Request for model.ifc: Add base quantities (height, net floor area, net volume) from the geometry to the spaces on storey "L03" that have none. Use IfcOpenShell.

First a look at what the model holds.

```python
import ifcopenshell
import ifcopenshell.util.element
import ifcopenshell.util.unit

model = ifcopenshell.open("model.ifc")
print(model.schema)
for unit_type in ("LENGTHUNIT", "AREAUNIT", "VOLUMEUNIT"):
    print(unit_type, ifcopenshell.util.unit.calculate_unit_scale(model, unit_type))
storey = next(s for s in model.by_type("IfcBuildingStorey") if s.Name == "L03")
spaces = [e for e in ifcopenshell.util.element.get_decomposition(storey) if e.is_a("IfcSpace")]
for e in sorted(spaces, key=lambda e: e.id()):
    print(e.id(), e.is_a(), e.Name, list(ifcopenshell.util.element.get_psets(e, qtos_only=True)), sep=" | ")
```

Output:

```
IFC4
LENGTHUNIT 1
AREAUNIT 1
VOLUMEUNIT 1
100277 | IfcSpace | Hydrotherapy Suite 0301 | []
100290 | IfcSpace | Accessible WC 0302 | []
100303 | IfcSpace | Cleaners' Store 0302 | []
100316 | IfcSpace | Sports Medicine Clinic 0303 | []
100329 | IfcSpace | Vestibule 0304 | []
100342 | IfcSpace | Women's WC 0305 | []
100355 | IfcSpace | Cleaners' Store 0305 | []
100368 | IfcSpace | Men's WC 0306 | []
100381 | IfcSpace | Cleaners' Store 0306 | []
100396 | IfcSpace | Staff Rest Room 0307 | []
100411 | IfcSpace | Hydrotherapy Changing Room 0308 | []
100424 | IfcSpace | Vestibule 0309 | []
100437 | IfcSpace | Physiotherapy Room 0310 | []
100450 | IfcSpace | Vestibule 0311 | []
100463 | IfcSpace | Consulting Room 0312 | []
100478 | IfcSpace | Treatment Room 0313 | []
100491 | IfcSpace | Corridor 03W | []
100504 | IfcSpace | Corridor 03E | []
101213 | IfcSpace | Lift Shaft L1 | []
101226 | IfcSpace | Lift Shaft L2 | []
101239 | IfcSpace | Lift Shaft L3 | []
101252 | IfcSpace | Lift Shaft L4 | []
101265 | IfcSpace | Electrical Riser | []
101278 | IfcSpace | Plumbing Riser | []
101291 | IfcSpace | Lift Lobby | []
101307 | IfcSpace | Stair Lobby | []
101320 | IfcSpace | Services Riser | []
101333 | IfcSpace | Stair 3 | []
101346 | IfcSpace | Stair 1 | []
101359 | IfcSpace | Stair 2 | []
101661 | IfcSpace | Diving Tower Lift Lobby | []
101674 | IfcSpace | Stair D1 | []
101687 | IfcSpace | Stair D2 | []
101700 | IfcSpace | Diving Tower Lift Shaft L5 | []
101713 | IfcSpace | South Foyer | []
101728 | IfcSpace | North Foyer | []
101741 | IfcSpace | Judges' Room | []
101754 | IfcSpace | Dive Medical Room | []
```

```python
import ifcopenshell
import ifcopenshell.api.pset
import ifcopenshell.geom
import ifcopenshell.util.element
import ifcopenshell.util.shape
import ifcopenshell.util.unit

model = ifcopenshell.open("model.ifc")
unit_scale = ifcopenshell.util.unit.calculate_unit_scale(model)
area_scale = ifcopenshell.util.unit.calculate_unit_scale(model, "AREAUNIT")
volume_scale = ifcopenshell.util.unit.calculate_unit_scale(model, "VOLUMEUNIT")
settings = ifcopenshell.geom.settings()

storey = next(s for s in model.by_type("IfcBuildingStorey") if s.Name == "L03")
spaces = [e for e in ifcopenshell.util.element.get_decomposition(storey) if e.is_a("IfcSpace")]

for e in sorted(spaces, key=lambda e: e.id()):
    if ifcopenshell.util.element.get_psets(e, qtos_only=True, should_inherit=False):
        continue
    # Geometry comes back in metres, in the element's own axes.
    shape = ifcopenshell.geom.create_shape(settings, e)
    values = {
        "Height": ifcopenshell.util.shape.get_z(shape.geometry) / unit_scale,
        "NetFloorArea": ifcopenshell.util.shape.get_footprint_area(shape.geometry) / area_scale,
        "NetVolume": ifcopenshell.util.shape.get_volume(shape.geometry) / volume_scale,
    }
    qto = ifcopenshell.api.pset.add_qto(model, product=e, name="Qto_SpaceBaseQuantities")
    ifcopenshell.api.pset.edit_qto(model, qto=qto, properties=values)
    print(e.id(), {k: round(v, 3) for k, v in values.items()})

model.write("model_v2.ifc")
```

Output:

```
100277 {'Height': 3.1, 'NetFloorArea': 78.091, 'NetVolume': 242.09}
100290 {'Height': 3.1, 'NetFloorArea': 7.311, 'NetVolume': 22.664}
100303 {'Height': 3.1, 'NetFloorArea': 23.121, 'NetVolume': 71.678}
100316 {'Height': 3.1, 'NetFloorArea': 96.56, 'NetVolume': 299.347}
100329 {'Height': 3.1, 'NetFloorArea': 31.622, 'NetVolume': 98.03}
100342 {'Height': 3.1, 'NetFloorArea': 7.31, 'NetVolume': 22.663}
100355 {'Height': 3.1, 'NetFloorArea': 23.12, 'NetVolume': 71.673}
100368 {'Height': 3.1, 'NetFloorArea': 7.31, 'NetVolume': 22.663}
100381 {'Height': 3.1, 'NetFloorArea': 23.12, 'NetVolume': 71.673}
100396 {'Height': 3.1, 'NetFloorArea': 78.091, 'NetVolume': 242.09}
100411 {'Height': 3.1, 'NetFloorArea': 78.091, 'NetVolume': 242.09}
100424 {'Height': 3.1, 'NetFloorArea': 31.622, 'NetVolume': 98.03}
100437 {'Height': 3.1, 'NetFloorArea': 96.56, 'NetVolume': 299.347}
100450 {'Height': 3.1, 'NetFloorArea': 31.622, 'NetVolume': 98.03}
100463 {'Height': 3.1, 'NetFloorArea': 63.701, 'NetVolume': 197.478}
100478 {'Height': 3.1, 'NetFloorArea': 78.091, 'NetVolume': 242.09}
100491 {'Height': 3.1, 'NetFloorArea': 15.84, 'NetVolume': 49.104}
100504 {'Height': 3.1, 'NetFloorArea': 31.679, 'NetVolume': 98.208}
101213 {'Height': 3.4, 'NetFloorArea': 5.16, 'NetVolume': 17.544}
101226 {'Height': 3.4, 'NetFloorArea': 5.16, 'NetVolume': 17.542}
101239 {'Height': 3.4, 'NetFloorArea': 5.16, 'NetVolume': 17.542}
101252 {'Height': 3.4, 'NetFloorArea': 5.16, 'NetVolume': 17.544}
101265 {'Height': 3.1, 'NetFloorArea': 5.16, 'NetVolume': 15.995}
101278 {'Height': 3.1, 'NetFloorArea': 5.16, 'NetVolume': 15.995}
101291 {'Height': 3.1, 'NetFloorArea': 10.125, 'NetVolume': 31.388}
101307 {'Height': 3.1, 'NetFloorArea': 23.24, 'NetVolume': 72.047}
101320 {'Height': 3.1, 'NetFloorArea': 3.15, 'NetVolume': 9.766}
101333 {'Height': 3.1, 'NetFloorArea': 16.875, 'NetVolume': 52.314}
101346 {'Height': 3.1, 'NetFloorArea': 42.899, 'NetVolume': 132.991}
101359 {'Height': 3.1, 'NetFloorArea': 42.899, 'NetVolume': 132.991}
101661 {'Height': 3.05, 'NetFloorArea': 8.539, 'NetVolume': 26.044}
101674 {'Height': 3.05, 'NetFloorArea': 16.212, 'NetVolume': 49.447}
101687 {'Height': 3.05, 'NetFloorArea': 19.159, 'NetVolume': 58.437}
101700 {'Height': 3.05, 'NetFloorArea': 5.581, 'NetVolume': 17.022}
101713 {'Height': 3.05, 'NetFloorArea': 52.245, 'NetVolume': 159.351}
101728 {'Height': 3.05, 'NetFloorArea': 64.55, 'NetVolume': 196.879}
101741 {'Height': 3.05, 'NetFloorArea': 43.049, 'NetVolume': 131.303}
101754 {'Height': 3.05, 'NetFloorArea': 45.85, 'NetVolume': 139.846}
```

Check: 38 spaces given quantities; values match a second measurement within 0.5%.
